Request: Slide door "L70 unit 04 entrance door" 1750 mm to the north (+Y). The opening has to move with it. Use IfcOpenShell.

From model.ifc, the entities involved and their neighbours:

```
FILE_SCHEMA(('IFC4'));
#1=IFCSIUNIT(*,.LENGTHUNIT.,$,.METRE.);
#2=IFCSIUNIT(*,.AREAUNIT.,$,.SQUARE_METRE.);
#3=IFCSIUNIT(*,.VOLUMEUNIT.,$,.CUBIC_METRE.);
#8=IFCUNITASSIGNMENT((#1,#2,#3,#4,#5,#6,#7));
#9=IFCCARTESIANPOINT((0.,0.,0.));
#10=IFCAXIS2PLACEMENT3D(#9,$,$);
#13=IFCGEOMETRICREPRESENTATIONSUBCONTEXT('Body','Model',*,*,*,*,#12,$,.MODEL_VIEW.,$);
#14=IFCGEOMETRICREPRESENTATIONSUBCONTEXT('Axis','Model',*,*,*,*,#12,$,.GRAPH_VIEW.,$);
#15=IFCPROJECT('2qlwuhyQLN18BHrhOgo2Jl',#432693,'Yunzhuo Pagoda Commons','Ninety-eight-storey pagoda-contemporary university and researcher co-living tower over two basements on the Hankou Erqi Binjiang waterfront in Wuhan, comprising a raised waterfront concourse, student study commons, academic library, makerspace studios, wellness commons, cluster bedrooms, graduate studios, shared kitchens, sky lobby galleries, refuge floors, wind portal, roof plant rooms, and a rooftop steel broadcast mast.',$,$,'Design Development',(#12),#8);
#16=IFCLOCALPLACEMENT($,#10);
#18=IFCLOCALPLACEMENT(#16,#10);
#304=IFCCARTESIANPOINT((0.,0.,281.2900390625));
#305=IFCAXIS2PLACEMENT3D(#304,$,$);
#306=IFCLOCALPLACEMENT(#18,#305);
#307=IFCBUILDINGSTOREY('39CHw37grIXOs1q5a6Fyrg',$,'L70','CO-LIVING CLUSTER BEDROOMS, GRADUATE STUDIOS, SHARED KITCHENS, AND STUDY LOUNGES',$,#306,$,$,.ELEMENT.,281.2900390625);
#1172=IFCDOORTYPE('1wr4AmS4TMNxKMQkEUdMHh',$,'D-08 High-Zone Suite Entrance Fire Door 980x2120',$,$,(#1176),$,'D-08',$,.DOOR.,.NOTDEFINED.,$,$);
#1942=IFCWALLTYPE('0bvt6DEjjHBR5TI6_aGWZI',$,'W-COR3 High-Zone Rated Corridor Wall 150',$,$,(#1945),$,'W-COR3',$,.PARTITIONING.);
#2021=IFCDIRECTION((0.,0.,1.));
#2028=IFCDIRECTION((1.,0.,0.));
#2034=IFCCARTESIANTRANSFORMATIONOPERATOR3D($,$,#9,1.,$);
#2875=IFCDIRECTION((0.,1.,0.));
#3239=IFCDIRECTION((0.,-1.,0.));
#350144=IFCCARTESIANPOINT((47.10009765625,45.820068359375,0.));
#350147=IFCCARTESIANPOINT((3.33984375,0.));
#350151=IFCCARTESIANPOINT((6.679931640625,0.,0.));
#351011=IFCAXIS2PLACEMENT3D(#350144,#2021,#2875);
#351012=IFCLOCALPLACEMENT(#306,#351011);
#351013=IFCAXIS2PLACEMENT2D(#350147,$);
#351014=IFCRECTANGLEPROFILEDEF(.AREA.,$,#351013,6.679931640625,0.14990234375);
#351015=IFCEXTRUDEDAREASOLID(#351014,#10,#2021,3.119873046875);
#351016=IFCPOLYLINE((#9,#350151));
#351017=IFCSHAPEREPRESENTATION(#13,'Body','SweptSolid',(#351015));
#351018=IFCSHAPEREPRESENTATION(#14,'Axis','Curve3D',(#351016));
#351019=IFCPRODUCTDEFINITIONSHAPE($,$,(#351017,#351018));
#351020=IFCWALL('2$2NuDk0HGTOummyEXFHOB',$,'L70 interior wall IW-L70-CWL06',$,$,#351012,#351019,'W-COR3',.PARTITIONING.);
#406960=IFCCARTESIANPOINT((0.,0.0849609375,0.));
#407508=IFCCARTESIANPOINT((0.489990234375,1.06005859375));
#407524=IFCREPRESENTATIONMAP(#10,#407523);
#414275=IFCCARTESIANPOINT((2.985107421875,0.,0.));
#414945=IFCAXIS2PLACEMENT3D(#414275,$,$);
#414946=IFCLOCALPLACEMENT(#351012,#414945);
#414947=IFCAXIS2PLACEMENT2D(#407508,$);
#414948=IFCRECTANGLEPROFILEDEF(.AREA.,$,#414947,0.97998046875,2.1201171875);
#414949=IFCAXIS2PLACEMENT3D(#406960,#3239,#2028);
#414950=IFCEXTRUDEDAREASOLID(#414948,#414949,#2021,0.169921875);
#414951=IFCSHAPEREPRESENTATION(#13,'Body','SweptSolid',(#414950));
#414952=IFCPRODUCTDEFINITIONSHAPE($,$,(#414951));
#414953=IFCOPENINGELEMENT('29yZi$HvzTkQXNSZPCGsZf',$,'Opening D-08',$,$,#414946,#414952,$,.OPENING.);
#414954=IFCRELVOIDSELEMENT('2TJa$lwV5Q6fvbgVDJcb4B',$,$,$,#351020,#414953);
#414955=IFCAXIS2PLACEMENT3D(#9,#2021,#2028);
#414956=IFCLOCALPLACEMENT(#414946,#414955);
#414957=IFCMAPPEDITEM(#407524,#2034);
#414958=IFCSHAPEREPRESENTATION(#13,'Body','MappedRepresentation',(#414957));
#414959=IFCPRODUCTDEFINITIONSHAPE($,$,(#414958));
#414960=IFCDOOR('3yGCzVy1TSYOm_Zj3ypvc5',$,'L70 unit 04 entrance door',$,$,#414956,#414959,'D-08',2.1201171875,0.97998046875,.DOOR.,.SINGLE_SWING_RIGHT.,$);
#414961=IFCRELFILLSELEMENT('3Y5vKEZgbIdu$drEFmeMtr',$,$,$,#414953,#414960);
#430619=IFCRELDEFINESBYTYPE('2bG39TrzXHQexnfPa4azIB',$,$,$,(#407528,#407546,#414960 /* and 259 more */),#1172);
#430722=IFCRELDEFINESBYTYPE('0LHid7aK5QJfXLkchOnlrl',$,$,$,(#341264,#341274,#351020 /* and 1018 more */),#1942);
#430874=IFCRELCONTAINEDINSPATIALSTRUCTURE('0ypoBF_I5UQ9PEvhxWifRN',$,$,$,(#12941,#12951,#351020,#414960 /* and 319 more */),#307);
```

```python
import ifcopenshell
import ifcopenshell.api.geometry
import ifcopenshell.util.placement

model = ifcopenshell.open("model.ifc")

door = model.by_guid("3yGCzVy1TSYOm_Zj3ypvc5")
opening = door.FillsVoids[0].RelatingOpeningElement
wall = opening.VoidsElements[0].RelatingBuildingElement

wall_matrix = ifcopenshell.util.placement.get_local_placement(wall.ObjectPlacement)
shift = wall_matrix[:3, 0] * 1.75
before = ifcopenshell.util.placement.get_local_placement(door.ObjectPlacement)[:3, 3].copy()

# The door is placed relative to its opening, so it follows when the opening moves.
matrix = ifcopenshell.util.placement.get_local_placement(opening.ObjectPlacement)
matrix[:3, 3] += shift
ifcopenshell.api.geometry.edit_object_placement(
    model, product=opening, matrix=matrix, is_si=False, should_transform_children=True
)

after = ifcopenshell.util.placement.get_local_placement(door.ObjectPlacement)[:3, 3]
print("door moved by", (after - before).round(3) + 0.0)

model.write("model_edited.ifc")
```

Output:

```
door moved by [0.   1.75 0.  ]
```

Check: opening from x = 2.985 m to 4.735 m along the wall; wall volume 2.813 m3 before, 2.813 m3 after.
